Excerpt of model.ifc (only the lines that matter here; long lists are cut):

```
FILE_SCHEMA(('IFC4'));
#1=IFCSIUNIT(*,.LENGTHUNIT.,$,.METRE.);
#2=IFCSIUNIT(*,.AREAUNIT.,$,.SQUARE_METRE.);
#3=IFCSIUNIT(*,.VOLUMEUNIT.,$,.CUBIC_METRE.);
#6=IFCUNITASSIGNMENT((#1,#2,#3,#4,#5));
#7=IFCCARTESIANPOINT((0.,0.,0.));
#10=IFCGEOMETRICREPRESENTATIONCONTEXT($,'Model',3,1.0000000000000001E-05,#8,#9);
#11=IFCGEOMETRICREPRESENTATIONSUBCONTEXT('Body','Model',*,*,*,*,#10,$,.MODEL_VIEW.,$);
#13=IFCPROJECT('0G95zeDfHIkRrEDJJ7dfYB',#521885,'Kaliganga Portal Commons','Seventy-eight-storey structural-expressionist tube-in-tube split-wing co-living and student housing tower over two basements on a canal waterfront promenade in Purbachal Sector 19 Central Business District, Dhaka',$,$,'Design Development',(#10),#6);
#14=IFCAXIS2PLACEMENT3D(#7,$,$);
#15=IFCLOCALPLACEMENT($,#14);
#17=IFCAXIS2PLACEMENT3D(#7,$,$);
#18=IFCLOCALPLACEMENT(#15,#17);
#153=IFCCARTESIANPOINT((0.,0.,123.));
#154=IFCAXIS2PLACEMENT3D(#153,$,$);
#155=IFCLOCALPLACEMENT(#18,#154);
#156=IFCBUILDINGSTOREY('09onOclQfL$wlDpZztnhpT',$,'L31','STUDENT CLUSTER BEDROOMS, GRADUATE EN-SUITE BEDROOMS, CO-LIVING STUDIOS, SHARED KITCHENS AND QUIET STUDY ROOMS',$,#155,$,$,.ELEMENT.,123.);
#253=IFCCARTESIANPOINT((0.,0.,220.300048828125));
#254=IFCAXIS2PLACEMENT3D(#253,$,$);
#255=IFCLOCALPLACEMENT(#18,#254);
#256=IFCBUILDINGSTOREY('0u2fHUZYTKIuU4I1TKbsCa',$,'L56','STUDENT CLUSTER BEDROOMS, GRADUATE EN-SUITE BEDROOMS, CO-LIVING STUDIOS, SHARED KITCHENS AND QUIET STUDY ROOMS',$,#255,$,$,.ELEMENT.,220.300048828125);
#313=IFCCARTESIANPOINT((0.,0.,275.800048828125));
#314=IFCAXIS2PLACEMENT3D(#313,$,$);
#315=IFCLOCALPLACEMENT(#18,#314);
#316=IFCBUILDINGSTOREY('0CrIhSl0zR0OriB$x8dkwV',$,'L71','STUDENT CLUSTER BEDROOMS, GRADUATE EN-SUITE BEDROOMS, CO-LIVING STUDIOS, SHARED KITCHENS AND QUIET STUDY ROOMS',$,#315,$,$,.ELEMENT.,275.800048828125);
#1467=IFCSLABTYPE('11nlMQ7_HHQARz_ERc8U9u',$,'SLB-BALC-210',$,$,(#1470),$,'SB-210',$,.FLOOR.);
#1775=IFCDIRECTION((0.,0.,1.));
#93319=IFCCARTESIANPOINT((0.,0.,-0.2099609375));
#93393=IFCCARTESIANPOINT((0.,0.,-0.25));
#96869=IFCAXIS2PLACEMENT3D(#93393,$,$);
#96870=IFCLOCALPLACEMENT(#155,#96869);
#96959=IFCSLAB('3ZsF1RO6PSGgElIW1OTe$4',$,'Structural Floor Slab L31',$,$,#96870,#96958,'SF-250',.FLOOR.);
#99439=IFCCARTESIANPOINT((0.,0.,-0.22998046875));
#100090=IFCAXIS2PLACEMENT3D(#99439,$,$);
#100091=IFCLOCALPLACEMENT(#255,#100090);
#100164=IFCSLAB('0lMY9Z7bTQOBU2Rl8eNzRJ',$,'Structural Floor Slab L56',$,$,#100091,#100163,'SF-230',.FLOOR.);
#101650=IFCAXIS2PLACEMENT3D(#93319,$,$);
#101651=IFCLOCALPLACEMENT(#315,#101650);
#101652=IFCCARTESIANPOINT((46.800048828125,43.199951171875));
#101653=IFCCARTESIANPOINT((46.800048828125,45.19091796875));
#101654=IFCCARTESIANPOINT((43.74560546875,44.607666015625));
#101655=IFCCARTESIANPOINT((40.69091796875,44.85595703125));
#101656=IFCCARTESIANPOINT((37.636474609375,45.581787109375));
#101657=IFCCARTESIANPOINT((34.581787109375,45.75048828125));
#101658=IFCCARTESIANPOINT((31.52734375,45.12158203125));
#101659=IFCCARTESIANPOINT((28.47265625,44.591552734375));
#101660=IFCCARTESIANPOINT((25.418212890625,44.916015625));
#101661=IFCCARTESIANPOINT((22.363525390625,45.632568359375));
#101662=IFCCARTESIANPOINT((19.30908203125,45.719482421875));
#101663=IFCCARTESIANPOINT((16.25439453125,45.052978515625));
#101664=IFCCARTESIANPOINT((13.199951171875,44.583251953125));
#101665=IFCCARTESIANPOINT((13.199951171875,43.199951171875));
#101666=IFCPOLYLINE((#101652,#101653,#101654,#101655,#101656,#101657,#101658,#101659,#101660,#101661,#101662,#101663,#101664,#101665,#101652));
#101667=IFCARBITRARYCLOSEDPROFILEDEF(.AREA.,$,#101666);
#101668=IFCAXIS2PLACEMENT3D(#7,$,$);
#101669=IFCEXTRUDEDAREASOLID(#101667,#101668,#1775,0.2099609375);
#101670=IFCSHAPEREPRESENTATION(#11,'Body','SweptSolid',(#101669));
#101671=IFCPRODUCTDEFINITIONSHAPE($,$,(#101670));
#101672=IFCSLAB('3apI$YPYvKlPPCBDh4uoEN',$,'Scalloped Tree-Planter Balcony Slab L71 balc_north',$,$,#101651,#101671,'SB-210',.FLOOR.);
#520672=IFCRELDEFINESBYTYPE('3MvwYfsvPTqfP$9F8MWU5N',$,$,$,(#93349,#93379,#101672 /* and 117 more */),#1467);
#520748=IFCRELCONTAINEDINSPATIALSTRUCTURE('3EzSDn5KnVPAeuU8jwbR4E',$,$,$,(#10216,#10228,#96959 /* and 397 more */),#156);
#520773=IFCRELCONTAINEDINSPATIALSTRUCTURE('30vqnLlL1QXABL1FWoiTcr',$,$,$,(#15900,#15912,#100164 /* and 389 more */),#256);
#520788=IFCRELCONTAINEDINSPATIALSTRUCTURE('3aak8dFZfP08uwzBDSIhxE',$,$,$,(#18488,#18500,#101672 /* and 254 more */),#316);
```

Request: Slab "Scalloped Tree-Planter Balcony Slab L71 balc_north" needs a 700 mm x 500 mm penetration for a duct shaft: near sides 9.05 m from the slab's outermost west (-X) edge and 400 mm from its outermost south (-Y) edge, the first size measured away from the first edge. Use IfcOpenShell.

```python
import numpy as np
import ifcopenshell
import ifcopenshell.api.feature
import ifcopenshell.api.geometry
import ifcopenshell.api.root
import ifcopenshell.geom
import ifcopenshell.util.placement
import ifcopenshell.util.representation
import ifcopenshell.util.shape
import ifcopenshell.util.unit

model = ifcopenshell.open("model.ifc")
unit_scale = ifcopenshell.util.unit.calculate_unit_scale(model)
settings = ifcopenshell.geom.settings()


def volume(element):
    """Net volume in cubic metres, openings subtracted."""
    shape = ifcopenshell.geom.create_shape(settings, element)
    return ifcopenshell.util.shape.get_volume(shape.geometry)


slab = model.by_guid("3apI$YPYvKlPPCBDh4uoEN")
before = volume(slab)

# Extent in the slab's own axes, in metres. The edges named are its -X and -Y sides.
slab_shape = ifcopenshell.geom.create_shape(settings, slab)
vertices = ifcopenshell.util.shape.get_vertices(slab_shape.geometry)
x_min, y_min, bottom = vertices.min(axis=0)
top = vertices[:, 2].max()

opening = ifcopenshell.api.root.create_entity(model, ifc_class="IfcOpeningElement", name="Duct shaft opening", predefined_type="OPENING")
context = ifcopenshell.util.representation.get_context(model, "Model", "Body", "MODEL_VIEW")
width, depth = 0.7, 0.5
outline = [(0.0, 0.0), (width, 0.0), (width, depth), (0.0, depth), (0.0, 0.0)]
# Overshoot both faces by 50 mm so the cut is clean.
shape = ifcopenshell.api.geometry.add_slab_representation(
    model, context=context, depth=top - bottom + 0.1, polyline=outline
)
ifcopenshell.api.geometry.assign_representation(model, product=opening, representation=shape)

matrix = ifcopenshell.util.placement.get_local_placement(slab.ObjectPlacement)
matrix[:, 3] = matrix @ np.append(np.array([x_min + 9.05, y_min + 0.4, bottom - 0.05]) / unit_scale, 1.0)
ifcopenshell.api.geometry.edit_object_placement(model, product=opening, matrix=matrix, is_si=False)
ifcopenshell.api.feature.add_feature(model, feature=opening, element=slab)

after = volume(slab)

print(f"slab volume {before:.3f} -> {after:.3f} m3")

model.write("model-out.ifc")
```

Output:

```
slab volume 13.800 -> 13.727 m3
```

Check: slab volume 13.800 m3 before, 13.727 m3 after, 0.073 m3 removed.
